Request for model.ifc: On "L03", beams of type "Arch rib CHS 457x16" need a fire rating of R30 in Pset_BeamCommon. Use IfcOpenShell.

First a look at what the model holds.

```python
import ifcopenshell
import ifcopenshell.util.element

model = ifcopenshell.open("model.ifc")
print(model.schema)
storey = next(s for s in model.by_type("IfcBuildingStorey") if s.Name == "L03")
beams = [e for e in ifcopenshell.util.element.get_decomposition(storey) if e.is_a("IfcBeam")]
seen = {}
for e in beams:
    element_type = ifcopenshell.util.element.get_type(e)
    key = (element_type.Name if element_type != e and element_type else None, ifcopenshell.util.element.get_pset(e, "Pset_BeamCommon", "FireRating"))
    seen[key] = seen.get(key, 0) + 1
for (name, value), count in sorted(seen.items(), key=str):
    print(count, "x", name, "|", value)
```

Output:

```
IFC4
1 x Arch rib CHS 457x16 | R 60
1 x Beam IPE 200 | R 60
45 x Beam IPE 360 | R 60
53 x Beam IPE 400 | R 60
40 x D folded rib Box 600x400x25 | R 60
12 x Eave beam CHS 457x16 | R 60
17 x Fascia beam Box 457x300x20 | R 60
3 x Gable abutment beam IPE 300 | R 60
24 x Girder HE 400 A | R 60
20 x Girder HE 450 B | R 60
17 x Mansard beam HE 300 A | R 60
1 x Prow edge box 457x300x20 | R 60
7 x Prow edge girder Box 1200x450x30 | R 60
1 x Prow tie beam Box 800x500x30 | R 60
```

```python
import ifcopenshell
import ifcopenshell.api.pset
import ifcopenshell.util.element

model = ifcopenshell.open("model.ifc")

storey = next(s for s in model.by_type("IfcBuildingStorey") if s.Name == "L03")
beams = [e for e in ifcopenshell.util.element.get_decomposition(storey) if e.is_a("IfcBeam")]

count = 0
for e in beams:
    element_type = ifcopenshell.util.element.get_type(e)
    if element_type in (None, e) or element_type.Name != "Arch rib CHS 457x16":
        continue
    # add_pset returns the element's existing set when there is one.
    pset = ifcopenshell.api.pset.add_pset(model, product=e, name="Pset_BeamCommon")
    ifcopenshell.api.pset.edit_pset(model, pset=pset, properties={"FireRating": "R30"})
    count += 1

print(count, "beams updated")

model.write("model_edited.ifc")
```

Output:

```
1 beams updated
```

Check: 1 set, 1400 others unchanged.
